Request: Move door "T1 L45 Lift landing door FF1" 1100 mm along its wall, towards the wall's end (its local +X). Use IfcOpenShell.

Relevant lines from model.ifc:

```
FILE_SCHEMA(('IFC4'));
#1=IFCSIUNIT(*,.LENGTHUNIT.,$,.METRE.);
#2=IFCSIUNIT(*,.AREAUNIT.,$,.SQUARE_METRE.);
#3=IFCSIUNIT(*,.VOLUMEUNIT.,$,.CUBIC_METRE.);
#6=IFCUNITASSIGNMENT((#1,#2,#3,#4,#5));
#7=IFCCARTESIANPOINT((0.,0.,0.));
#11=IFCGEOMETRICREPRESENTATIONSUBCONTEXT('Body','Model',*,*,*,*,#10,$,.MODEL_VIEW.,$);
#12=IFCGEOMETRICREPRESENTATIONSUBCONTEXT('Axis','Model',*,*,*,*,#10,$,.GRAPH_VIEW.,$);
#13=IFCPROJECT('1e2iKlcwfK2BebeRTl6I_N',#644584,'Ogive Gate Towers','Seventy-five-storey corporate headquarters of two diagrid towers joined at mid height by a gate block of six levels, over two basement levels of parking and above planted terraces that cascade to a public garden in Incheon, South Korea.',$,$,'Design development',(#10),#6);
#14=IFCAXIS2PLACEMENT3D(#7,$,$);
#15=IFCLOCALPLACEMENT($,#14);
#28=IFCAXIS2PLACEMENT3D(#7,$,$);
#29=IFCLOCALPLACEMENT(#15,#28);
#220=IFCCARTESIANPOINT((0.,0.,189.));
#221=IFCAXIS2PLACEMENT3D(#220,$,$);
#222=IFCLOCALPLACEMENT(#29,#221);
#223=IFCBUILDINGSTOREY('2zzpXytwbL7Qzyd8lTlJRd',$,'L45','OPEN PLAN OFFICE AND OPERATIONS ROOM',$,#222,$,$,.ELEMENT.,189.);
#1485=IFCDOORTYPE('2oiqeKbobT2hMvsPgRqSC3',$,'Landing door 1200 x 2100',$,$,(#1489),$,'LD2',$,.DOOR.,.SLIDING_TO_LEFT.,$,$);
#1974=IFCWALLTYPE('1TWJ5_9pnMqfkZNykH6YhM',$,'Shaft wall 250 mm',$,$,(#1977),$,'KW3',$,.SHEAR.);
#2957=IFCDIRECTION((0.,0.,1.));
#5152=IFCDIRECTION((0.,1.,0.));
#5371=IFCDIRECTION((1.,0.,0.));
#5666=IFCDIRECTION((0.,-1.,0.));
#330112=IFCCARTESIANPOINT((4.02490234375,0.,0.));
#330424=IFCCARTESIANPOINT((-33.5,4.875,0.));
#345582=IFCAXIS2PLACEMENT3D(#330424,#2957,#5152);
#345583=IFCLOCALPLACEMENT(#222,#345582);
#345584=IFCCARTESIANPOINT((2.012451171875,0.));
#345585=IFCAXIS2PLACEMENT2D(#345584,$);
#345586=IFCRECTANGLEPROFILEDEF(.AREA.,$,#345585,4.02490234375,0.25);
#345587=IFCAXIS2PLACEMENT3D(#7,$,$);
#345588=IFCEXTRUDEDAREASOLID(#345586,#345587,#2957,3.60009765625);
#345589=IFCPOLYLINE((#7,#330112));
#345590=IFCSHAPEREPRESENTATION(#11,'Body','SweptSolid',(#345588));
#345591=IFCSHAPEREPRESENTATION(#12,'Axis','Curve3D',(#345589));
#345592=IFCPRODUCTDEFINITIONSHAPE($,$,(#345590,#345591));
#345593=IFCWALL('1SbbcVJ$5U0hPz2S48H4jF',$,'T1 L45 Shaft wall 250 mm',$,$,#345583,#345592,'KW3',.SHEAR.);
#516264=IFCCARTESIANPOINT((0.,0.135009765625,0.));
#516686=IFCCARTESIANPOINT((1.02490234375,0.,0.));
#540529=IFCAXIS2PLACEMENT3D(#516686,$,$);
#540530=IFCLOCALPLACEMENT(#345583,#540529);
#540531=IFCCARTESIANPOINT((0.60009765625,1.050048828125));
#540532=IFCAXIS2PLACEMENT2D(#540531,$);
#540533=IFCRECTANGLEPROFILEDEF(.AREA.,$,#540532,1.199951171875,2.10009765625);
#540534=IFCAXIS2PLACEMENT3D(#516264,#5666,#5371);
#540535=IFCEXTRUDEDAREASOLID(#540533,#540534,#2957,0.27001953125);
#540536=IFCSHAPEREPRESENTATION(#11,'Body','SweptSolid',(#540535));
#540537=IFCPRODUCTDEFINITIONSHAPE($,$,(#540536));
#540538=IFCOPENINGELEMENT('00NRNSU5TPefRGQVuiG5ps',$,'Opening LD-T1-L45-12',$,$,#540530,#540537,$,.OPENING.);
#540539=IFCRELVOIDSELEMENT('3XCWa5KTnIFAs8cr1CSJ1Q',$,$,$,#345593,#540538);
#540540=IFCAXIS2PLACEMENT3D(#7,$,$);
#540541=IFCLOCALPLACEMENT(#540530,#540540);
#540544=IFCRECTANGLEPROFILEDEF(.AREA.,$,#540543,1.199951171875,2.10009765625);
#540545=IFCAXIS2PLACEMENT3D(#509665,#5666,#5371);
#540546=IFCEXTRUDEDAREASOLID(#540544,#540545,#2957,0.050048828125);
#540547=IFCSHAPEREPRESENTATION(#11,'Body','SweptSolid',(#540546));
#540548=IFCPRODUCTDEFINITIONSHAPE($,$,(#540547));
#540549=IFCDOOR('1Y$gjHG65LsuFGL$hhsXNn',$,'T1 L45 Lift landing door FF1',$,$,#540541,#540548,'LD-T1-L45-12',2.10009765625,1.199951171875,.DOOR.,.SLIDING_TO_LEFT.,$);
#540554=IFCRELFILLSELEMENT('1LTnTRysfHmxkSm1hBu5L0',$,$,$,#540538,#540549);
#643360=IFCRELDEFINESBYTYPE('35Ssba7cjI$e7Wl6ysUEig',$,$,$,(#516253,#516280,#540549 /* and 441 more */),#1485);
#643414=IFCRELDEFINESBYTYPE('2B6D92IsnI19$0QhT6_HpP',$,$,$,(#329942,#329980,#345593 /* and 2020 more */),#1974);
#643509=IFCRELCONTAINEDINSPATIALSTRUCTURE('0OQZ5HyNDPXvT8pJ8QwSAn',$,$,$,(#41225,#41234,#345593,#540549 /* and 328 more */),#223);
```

```python
import ifcopenshell
import ifcopenshell.api.geometry
import ifcopenshell.util.placement
import ifcopenshell.util.unit

model = ifcopenshell.open("model.ifc")
unit_scale = ifcopenshell.util.unit.calculate_unit_scale(model)

door = model.by_guid("1Y$gjHG65LsuFGL$hhsXNn")
opening = door.FillsVoids[0].RelatingOpeningElement
wall = opening.VoidsElements[0].RelatingBuildingElement

wall_matrix = ifcopenshell.util.placement.get_local_placement(wall.ObjectPlacement)
shift = wall_matrix[:3, 0] * 1.1 / unit_scale
before = ifcopenshell.util.placement.get_local_placement(door.ObjectPlacement)[:3, 3].copy()

# The door is placed relative to its opening, so it follows when the opening moves.
matrix = ifcopenshell.util.placement.get_local_placement(opening.ObjectPlacement)
matrix[:3, 3] += shift
ifcopenshell.api.geometry.edit_object_placement(
    model, product=opening, matrix=matrix, is_si=False, should_transform_children=True
)

after = ifcopenshell.util.placement.get_local_placement(door.ObjectPlacement)[:3, 3]
print("door moved by", (after - before).round(3) + 0.0)

model.write("model_updated.ifc")
```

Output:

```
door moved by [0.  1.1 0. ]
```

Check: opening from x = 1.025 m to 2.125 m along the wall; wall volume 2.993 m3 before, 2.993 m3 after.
